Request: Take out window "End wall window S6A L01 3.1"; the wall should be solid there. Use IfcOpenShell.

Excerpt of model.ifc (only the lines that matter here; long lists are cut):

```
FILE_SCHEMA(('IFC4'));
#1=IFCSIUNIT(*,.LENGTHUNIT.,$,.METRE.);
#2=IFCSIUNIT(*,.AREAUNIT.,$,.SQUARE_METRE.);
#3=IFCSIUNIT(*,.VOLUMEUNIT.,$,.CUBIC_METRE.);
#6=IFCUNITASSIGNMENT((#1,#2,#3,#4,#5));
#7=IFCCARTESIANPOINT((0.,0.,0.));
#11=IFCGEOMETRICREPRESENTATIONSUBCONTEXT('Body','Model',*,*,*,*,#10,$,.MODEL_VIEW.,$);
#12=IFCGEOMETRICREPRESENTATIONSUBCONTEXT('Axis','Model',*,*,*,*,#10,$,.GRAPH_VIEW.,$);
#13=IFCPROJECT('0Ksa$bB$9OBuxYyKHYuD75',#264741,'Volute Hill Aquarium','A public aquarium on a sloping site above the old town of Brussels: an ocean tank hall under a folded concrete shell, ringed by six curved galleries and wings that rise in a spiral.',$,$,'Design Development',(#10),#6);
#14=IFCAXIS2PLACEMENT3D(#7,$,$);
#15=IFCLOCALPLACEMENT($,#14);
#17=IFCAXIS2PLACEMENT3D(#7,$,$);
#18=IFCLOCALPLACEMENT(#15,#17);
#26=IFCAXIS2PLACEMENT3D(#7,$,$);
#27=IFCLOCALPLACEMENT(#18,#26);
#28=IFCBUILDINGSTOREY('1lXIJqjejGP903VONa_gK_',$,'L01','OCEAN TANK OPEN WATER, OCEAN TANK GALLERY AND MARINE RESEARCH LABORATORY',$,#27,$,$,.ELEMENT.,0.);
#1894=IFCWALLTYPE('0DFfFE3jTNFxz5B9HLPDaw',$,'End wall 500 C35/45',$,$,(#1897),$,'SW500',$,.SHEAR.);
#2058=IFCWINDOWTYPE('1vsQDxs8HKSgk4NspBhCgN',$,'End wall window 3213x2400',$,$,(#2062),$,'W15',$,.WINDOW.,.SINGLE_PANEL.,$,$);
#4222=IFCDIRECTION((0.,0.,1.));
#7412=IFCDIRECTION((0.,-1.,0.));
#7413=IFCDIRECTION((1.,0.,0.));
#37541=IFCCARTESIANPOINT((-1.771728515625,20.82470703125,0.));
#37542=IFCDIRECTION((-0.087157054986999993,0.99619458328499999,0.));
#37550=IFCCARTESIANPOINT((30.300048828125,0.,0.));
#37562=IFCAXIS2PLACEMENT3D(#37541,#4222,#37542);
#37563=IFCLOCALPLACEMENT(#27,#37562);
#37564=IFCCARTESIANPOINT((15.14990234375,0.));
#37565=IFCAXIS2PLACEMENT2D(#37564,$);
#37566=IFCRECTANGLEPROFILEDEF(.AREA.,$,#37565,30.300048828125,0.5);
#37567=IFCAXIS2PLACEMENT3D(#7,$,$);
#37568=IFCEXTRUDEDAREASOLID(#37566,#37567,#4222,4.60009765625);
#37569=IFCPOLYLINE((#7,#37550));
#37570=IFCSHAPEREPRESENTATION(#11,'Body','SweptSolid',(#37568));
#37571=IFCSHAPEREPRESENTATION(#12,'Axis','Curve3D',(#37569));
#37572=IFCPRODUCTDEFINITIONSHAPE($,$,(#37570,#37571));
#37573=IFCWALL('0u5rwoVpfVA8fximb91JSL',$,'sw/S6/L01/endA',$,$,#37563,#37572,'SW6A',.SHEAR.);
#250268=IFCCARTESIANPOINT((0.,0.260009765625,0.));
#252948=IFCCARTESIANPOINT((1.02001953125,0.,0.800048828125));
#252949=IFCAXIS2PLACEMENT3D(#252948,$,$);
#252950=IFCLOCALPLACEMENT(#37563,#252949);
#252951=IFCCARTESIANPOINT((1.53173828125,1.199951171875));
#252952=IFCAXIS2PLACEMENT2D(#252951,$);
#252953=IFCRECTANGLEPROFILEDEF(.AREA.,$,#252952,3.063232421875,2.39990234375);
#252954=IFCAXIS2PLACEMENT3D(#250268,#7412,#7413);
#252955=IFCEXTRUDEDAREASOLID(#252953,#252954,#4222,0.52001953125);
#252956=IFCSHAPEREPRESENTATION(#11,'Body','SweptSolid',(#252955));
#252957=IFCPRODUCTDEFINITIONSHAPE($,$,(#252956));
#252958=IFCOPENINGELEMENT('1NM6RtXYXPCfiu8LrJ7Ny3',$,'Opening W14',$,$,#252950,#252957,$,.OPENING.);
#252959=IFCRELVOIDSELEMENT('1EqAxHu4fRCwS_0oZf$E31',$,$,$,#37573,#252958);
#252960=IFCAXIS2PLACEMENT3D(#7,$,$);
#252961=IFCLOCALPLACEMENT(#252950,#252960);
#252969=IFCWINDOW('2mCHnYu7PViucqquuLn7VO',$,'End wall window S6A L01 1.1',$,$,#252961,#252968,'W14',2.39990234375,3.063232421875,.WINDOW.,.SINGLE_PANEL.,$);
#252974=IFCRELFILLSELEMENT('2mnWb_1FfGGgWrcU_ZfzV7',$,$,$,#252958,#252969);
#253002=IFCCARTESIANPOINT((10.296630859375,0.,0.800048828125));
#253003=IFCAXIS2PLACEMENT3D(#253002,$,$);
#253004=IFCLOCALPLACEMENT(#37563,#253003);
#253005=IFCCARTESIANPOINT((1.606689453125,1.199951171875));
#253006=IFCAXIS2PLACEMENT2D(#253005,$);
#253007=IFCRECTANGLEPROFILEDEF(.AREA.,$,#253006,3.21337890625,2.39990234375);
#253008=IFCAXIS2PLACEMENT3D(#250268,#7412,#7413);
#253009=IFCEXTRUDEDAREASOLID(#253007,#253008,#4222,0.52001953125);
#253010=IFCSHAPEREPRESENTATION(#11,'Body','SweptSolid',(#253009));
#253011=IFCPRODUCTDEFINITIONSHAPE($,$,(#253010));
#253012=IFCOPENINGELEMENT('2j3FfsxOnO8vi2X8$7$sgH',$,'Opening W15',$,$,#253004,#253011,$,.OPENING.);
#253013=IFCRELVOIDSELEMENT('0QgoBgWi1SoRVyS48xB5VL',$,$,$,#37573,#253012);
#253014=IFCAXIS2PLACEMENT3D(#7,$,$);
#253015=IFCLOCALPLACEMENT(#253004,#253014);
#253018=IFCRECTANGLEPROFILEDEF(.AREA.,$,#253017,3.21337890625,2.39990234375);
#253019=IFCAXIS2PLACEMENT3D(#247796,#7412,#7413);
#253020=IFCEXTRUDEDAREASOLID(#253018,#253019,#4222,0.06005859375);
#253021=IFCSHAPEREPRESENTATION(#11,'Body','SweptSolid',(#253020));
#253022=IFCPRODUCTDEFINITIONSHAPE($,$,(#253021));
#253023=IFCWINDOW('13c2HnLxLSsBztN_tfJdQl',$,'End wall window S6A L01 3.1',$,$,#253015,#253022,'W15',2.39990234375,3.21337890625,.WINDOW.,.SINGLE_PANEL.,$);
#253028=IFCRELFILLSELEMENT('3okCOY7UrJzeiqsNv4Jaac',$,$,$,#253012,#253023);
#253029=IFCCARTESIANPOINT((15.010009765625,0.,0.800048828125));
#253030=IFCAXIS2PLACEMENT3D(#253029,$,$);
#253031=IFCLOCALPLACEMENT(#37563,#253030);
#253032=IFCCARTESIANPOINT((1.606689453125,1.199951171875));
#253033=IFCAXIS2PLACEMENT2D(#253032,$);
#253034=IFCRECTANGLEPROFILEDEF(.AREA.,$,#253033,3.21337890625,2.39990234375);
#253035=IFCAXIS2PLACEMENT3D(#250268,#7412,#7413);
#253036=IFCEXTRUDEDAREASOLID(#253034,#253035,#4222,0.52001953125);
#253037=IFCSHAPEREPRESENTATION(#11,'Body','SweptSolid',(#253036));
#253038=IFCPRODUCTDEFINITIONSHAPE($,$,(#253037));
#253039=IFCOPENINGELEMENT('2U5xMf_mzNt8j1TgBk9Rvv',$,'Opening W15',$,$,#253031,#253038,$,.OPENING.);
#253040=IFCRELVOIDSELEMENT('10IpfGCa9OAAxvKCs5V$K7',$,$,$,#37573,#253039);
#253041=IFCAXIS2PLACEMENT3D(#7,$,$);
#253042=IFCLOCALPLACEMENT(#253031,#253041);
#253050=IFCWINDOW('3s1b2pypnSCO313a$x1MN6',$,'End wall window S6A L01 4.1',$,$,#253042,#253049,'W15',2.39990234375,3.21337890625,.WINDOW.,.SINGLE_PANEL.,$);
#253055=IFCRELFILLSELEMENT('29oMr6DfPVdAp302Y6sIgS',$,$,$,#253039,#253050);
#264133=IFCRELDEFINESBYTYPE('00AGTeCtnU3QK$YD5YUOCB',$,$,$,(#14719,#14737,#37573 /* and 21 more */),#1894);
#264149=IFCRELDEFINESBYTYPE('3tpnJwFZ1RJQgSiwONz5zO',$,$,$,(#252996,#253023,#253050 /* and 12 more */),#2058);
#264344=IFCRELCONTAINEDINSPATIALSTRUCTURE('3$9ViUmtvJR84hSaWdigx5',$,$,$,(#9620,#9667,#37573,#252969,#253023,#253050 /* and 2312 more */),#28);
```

```python
import ifcopenshell
import ifcopenshell.api.feature
import ifcopenshell.api.root
import ifcopenshell.geom
import ifcopenshell.util.shape

model = ifcopenshell.open("model.ifc")
settings = ifcopenshell.geom.settings()


def volume(element):
    """Net volume in cubic metres, openings subtracted."""
    shape = ifcopenshell.geom.create_shape(settings, element)
    return ifcopenshell.util.shape.get_volume(shape.geometry)


window = model.by_id(253023)
opening = window.FillsVoids[0].RelatingOpeningElement
wall = opening.VoidsElements[0].RelatingBuildingElement
before = volume(wall)

ifcopenshell.api.root.remove_product(model, product=window)
ifcopenshell.api.feature.remove_feature(model, feature=opening)

after = volume(wall)

print(f"wall volume {before:.3f} -> {after:.3f} m3")

model.write("model-out.ifc")
```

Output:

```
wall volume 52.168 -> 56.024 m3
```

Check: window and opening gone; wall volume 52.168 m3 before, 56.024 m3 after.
